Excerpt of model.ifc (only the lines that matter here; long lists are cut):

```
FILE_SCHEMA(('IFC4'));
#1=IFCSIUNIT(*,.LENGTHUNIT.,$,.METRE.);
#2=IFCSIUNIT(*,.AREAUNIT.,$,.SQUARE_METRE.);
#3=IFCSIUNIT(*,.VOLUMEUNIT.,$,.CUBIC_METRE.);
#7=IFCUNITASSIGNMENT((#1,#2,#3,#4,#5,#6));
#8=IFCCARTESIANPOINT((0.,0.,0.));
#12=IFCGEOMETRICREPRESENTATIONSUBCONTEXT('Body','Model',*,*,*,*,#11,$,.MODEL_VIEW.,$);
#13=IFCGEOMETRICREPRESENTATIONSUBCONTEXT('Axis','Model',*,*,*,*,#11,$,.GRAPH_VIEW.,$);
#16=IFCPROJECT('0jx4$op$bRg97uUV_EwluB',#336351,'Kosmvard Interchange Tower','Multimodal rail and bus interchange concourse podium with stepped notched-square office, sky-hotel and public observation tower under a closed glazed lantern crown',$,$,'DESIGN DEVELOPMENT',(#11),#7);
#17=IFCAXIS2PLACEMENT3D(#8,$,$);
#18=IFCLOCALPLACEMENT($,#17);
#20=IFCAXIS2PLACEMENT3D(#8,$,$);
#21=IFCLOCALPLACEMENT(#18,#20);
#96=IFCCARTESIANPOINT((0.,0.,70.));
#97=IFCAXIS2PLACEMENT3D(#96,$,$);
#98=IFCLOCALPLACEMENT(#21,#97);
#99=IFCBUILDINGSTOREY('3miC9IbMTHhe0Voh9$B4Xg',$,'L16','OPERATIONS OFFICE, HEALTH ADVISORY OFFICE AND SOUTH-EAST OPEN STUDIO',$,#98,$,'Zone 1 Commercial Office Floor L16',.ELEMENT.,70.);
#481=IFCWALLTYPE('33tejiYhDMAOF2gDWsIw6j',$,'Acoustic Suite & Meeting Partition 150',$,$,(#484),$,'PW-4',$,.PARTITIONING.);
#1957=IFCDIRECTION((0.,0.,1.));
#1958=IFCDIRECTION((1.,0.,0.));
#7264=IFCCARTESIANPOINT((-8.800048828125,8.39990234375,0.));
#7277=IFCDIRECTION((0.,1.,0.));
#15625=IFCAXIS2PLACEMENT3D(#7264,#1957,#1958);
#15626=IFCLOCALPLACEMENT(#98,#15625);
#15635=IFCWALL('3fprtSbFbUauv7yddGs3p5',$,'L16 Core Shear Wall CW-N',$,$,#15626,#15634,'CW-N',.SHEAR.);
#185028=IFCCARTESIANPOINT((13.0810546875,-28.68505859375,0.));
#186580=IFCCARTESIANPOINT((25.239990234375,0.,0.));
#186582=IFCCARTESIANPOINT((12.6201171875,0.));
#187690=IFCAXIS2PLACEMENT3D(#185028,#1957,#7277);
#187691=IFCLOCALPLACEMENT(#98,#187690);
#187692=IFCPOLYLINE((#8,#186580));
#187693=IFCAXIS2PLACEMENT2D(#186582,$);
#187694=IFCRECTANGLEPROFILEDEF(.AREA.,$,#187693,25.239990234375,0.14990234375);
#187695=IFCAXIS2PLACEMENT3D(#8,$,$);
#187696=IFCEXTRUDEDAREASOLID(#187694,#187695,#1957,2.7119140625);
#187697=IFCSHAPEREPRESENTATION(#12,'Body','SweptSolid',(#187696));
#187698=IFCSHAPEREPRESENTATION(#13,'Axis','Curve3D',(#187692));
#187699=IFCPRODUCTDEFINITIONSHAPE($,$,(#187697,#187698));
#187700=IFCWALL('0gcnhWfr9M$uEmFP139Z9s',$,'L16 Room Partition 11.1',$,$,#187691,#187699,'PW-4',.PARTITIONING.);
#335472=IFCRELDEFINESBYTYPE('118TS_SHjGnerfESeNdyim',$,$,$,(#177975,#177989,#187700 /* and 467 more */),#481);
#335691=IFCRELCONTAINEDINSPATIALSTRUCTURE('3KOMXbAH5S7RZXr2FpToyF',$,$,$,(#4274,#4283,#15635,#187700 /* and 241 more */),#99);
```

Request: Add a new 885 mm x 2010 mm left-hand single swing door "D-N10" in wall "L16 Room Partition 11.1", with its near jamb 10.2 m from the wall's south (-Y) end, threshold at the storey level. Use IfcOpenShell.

```python
import numpy as np
import ifcopenshell
import ifcopenshell.api.feature
import ifcopenshell.api.geometry
import ifcopenshell.api.root
import ifcopenshell.api.spatial
import ifcopenshell.geom
import ifcopenshell.util.element
import ifcopenshell.util.placement
import ifcopenshell.util.representation
import ifcopenshell.util.shape
import ifcopenshell.util.unit

model = ifcopenshell.open("model.ifc")
unit_scale = ifcopenshell.util.unit.calculate_unit_scale(model)
settings = ifcopenshell.geom.settings()


def volume(element):
    """Net volume in cubic metres, openings subtracted."""
    shape = ifcopenshell.geom.create_shape(settings, element)
    return ifcopenshell.util.shape.get_volume(shape.geometry)


wall = model.by_id(187700)
storey = ifcopenshell.util.element.get_container(wall, ifc_class="IfcBuildingStorey")
context = ifcopenshell.util.representation.get_context(model, "Model", "Body", "MODEL_VIEW")
before = volume(wall)

width, height, from_end, sill = 0.885, 2.01, 10.2, 0.0  # metres

# The wall runs along its own X axis, and the end named is its -X end.
wall_shape = ifcopenshell.geom.create_shape(settings, wall)
x, y, z = ifcopenshell.util.shape.get_vertices(wall_shape.geometry).T
start = x.min() + from_end
face, thickness = float(y.min()), float(y.max() - y.min())
wall_matrix = ifcopenshell.util.placement.get_local_placement(wall.ObjectPlacement)
level = ifcopenshell.util.placement.get_local_placement(storey.ObjectPlacement)[2, 3]


def in_wall(x, y):
    """Placement at x, y metres in the wall's axes, at sill height."""
    matrix = wall_matrix.copy()
    matrix[:, 3] = wall_matrix @ np.array([x / unit_scale, y / unit_scale, 0.0, 1.0])
    matrix[2, 3] = level + sill / unit_scale
    return matrix


# Opening: a box that overshoots both wall faces by 50 mm.
opening = ifcopenshell.api.root.create_entity(model, ifc_class="IfcOpeningElement", predefined_type="OPENING")
box = ifcopenshell.api.geometry.add_wall_representation(
    model, context=context, length=width, height=height, thickness=thickness + 0.1
)
ifcopenshell.api.geometry.assign_representation(model, product=opening, representation=box)
ifcopenshell.api.geometry.edit_object_placement(model, product=opening, matrix=in_wall(start, face - 0.05), is_si=False)
ifcopenshell.api.feature.add_feature(model, feature=opening, element=wall)

door = ifcopenshell.api.root.create_entity(model, ifc_class="IfcDoor", name="D-N10", predefined_type="DOOR")
door.OverallWidth, door.OverallHeight = width / unit_scale, height / unit_scale
door.OperationType = "SINGLE_SWING_LEFT"
body = ifcopenshell.api.geometry.add_door_representation(
    model,
    context=context,
    overall_width=door.OverallWidth,
    overall_height=door.OverallHeight,
    operation_type="SINGLE_SWING_LEFT",
    lining_properties={"LiningDepth": thickness / unit_scale, "ThresholdDepth": thickness / unit_scale},
)
ifcopenshell.api.geometry.assign_representation(model, product=door, representation=body)
ifcopenshell.api.spatial.assign_container(model, products=[door], relating_structure=storey)
ifcopenshell.api.feature.add_filling(model, opening=opening, element=door)

# The lining spans the wall, so the door starts at the wall face.
ifcopenshell.api.geometry.edit_object_placement(model, product=door, matrix=in_wall(start, face), is_si=False)

after = volume(wall)

print(f"wall volume {before:.3f} -> {after:.3f} m3")

model.write("model-out.ifc")
```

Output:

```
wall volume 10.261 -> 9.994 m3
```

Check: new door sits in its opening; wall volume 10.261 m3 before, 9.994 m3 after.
